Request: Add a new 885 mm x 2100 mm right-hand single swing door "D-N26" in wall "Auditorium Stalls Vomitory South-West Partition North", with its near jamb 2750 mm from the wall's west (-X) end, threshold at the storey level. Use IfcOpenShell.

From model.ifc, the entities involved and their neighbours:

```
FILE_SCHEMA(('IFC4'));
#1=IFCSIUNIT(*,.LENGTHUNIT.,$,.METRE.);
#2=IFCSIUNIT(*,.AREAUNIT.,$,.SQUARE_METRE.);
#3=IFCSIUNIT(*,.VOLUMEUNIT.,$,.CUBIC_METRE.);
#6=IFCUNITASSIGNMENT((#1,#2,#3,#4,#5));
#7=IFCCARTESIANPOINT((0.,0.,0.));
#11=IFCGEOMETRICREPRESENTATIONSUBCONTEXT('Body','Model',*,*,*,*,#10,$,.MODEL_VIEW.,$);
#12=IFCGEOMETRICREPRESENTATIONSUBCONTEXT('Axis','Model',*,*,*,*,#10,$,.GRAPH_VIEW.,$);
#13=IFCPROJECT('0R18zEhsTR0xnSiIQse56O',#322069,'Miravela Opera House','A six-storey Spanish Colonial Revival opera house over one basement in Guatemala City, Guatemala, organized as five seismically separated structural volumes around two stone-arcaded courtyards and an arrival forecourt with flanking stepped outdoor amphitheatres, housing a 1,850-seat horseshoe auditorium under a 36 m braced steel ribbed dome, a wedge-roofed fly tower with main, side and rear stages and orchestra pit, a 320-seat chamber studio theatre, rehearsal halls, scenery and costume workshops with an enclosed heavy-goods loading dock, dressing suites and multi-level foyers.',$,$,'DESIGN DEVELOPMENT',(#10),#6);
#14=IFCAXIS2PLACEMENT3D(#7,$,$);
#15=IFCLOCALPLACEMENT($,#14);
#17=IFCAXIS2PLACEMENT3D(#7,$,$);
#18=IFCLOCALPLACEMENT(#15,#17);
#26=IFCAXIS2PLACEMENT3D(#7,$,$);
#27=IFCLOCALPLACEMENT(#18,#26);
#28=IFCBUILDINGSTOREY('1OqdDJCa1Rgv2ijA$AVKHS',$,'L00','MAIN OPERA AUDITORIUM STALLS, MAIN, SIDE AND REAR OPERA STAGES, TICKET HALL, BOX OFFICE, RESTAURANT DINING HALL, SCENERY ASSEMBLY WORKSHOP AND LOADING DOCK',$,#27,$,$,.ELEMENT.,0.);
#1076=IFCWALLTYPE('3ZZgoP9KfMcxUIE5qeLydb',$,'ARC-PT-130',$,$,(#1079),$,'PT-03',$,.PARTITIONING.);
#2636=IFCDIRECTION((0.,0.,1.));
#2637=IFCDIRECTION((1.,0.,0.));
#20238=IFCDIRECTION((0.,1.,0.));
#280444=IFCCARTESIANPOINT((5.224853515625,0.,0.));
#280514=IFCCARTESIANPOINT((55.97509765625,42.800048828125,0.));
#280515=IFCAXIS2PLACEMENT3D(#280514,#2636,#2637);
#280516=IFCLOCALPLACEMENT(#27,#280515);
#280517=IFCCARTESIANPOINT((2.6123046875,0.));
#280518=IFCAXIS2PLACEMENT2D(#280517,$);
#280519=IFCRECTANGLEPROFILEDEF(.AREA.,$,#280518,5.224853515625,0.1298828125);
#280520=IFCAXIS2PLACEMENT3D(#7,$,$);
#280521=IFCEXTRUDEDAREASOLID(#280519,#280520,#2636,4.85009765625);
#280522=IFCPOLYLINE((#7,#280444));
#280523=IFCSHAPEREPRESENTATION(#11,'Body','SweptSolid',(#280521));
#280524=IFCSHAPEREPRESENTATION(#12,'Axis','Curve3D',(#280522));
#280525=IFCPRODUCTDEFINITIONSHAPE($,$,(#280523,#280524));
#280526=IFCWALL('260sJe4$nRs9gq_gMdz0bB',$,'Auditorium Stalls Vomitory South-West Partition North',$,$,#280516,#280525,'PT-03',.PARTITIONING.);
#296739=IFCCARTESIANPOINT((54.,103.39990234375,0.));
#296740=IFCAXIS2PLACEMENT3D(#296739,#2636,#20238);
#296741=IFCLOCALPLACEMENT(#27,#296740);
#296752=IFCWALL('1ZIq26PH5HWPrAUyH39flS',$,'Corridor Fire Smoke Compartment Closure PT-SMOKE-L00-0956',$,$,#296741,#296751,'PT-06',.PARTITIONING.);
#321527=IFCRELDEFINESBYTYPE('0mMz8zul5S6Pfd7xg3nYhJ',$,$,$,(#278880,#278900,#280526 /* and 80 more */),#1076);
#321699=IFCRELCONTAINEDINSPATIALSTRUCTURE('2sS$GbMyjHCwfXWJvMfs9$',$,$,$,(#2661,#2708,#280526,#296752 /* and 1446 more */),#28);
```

```python
import numpy as np
import ifcopenshell
import ifcopenshell.api.feature
import ifcopenshell.api.geometry
import ifcopenshell.api.root
import ifcopenshell.api.spatial
import ifcopenshell.geom
import ifcopenshell.util.element
import ifcopenshell.util.placement
import ifcopenshell.util.representation
import ifcopenshell.util.shape
import ifcopenshell.util.unit

model = ifcopenshell.open("model.ifc")
unit_scale = ifcopenshell.util.unit.calculate_unit_scale(model)
settings = ifcopenshell.geom.settings()


def volume(element):
    """Net volume in cubic metres, openings subtracted."""
    shape = ifcopenshell.geom.create_shape(settings, element)
    return ifcopenshell.util.shape.get_volume(shape.geometry)


wall = model.by_guid("260sJe4$nRs9gq_gMdz0bB")
storey = ifcopenshell.util.element.get_container(wall, ifc_class="IfcBuildingStorey")
context = ifcopenshell.util.representation.get_context(model, "Model", "Body", "MODEL_VIEW")
before = volume(wall)

width, height, from_end, sill = 0.885, 2.1, 2.75, 0.0  # metres

# The wall runs along its own X axis, and the end named is its -X end.
wall_shape = ifcopenshell.geom.create_shape(settings, wall)
x, y, z = ifcopenshell.util.shape.get_vertices(wall_shape.geometry).T
start = x.min() + from_end
face, thickness = float(y.min()), float(y.max() - y.min())
wall_matrix = ifcopenshell.util.placement.get_local_placement(wall.ObjectPlacement)
level = ifcopenshell.util.placement.get_local_placement(storey.ObjectPlacement)[2, 3]


def in_wall(x, y):
    """Placement at x, y metres in the wall's axes, at sill height."""
    matrix = wall_matrix.copy()
    matrix[:, 3] = wall_matrix @ np.array([x / unit_scale, y / unit_scale, 0.0, 1.0])
    matrix[2, 3] = level + sill / unit_scale
    return matrix


# Opening: a box that overshoots both wall faces by 50 mm.
opening = ifcopenshell.api.root.create_entity(model, ifc_class="IfcOpeningElement", predefined_type="OPENING")
box = ifcopenshell.api.geometry.add_wall_representation(
    model, context=context, length=width, height=height, thickness=thickness + 0.1
)
ifcopenshell.api.geometry.assign_representation(model, product=opening, representation=box)
ifcopenshell.api.geometry.edit_object_placement(model, product=opening, matrix=in_wall(start, face - 0.05), is_si=False)
ifcopenshell.api.feature.add_feature(model, feature=opening, element=wall)

door = ifcopenshell.api.root.create_entity(model, ifc_class="IfcDoor", name="D-N26", predefined_type="DOOR")
door.OverallWidth, door.OverallHeight = width / unit_scale, height / unit_scale
door.OperationType = "SINGLE_SWING_RIGHT"
body = ifcopenshell.api.geometry.add_door_representation(
    model,
    context=context,
    overall_width=door.OverallWidth,
    overall_height=door.OverallHeight,
    operation_type="SINGLE_SWING_RIGHT",
    lining_properties={"LiningDepth": thickness / unit_scale, "ThresholdDepth": thickness / unit_scale},
)
ifcopenshell.api.geometry.assign_representation(model, product=door, representation=body)
ifcopenshell.api.spatial.assign_container(model, products=[door], relating_structure=storey)
ifcopenshell.api.feature.add_filling(model, opening=opening, element=door)

# The lining spans the wall, so the door starts at the wall face.
ifcopenshell.api.geometry.edit_object_placement(model, product=door, matrix=in_wall(start, face), is_si=False)

after = volume(wall)

print(f"wall volume {before:.3f} -> {after:.3f} m3")

model.write("model_v2.ifc")
```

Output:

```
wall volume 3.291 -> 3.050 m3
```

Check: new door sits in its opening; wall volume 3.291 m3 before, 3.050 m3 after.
